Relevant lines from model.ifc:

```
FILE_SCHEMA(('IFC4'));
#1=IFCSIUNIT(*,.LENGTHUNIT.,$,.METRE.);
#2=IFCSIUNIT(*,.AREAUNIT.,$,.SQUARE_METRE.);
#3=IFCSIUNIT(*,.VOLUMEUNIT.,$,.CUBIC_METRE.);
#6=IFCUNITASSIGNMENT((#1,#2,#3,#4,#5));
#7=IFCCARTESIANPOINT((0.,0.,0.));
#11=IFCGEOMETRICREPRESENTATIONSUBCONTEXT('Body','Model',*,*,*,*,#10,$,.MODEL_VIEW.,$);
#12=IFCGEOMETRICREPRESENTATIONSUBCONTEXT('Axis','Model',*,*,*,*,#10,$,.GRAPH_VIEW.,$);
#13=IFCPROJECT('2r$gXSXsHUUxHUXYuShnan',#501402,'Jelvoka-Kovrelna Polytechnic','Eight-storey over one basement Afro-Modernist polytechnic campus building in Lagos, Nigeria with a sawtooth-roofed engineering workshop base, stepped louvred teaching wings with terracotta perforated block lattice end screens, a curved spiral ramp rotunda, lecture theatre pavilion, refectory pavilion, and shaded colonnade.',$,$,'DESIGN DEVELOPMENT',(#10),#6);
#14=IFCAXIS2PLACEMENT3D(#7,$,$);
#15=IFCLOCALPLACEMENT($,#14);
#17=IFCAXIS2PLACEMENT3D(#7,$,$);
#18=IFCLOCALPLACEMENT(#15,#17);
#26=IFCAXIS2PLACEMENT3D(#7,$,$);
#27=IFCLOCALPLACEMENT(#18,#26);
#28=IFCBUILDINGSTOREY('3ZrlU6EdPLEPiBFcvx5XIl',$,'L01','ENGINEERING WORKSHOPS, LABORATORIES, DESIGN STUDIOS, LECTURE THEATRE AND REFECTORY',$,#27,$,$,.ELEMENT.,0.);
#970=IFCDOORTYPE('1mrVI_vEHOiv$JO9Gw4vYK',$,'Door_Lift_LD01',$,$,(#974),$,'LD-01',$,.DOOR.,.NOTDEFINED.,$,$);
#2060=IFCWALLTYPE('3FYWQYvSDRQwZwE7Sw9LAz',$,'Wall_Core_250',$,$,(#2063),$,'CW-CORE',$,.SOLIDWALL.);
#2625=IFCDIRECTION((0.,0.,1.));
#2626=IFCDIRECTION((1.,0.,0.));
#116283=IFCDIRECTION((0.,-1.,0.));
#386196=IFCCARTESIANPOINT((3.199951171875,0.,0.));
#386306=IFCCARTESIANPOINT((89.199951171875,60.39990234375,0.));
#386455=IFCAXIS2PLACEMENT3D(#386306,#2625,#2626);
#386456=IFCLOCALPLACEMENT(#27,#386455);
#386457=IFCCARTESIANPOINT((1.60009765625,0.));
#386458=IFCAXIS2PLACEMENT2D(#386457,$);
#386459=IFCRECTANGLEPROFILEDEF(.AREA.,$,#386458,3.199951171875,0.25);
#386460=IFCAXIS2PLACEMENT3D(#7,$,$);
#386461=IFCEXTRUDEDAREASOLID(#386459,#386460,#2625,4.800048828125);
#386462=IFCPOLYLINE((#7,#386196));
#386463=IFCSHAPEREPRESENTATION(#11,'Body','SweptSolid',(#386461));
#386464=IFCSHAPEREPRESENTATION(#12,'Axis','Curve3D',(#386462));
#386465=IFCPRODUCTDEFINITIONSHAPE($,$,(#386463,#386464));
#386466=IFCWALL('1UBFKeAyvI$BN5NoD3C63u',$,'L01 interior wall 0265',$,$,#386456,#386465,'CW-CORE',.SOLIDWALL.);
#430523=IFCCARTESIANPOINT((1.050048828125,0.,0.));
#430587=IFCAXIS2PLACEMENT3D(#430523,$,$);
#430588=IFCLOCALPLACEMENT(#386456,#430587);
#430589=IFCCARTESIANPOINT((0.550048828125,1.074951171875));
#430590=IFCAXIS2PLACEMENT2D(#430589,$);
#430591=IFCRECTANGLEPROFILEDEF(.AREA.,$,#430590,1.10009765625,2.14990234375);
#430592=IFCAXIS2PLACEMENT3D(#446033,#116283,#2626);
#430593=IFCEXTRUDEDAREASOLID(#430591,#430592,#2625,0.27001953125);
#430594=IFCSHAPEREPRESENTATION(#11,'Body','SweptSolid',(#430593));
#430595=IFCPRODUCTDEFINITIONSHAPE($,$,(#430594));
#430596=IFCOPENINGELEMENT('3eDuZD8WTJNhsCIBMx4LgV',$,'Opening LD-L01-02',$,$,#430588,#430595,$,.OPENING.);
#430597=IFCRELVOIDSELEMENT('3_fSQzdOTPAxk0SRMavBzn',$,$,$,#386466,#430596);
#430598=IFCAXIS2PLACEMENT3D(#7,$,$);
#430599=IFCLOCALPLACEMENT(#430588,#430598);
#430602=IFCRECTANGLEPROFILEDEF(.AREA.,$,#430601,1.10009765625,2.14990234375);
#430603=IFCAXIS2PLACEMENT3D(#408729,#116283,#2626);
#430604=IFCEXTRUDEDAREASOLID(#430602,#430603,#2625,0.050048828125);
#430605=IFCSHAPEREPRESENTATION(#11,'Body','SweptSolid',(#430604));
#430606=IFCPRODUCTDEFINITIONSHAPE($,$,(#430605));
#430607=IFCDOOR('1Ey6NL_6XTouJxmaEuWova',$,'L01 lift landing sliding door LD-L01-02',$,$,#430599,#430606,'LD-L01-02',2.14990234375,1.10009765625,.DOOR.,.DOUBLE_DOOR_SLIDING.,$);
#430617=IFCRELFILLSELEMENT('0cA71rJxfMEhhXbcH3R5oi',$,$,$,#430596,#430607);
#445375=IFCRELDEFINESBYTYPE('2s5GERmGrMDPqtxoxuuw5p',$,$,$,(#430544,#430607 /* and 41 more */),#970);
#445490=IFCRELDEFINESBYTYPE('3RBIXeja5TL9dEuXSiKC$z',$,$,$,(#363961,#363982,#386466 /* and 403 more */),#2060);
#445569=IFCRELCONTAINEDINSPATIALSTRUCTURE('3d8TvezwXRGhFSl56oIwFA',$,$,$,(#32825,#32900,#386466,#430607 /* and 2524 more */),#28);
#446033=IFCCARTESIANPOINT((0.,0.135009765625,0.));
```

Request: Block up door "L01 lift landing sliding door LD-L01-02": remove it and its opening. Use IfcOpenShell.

```python
import ifcopenshell
import ifcopenshell.api.feature
import ifcopenshell.api.root
import ifcopenshell.geom
import ifcopenshell.util.shape

model = ifcopenshell.open("model.ifc")
settings = ifcopenshell.geom.settings()


def volume(element):
    """Net volume in cubic metres, openings subtracted."""
    shape = ifcopenshell.geom.create_shape(settings, element)
    return ifcopenshell.util.shape.get_volume(shape.geometry)


door = model.by_guid("1Ey6NL_6XTouJxmaEuWova")
opening = door.FillsVoids[0].RelatingOpeningElement
wall = opening.VoidsElements[0].RelatingBuildingElement
before = volume(wall)

ifcopenshell.api.root.remove_product(model, product=door)
ifcopenshell.api.feature.remove_feature(model, feature=opening)

after = volume(wall)

print(f"wall volume {before:.3f} -> {after:.3f} m3")

model.write("model_updated.ifc")
```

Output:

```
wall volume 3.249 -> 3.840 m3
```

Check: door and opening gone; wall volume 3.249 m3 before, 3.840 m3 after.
